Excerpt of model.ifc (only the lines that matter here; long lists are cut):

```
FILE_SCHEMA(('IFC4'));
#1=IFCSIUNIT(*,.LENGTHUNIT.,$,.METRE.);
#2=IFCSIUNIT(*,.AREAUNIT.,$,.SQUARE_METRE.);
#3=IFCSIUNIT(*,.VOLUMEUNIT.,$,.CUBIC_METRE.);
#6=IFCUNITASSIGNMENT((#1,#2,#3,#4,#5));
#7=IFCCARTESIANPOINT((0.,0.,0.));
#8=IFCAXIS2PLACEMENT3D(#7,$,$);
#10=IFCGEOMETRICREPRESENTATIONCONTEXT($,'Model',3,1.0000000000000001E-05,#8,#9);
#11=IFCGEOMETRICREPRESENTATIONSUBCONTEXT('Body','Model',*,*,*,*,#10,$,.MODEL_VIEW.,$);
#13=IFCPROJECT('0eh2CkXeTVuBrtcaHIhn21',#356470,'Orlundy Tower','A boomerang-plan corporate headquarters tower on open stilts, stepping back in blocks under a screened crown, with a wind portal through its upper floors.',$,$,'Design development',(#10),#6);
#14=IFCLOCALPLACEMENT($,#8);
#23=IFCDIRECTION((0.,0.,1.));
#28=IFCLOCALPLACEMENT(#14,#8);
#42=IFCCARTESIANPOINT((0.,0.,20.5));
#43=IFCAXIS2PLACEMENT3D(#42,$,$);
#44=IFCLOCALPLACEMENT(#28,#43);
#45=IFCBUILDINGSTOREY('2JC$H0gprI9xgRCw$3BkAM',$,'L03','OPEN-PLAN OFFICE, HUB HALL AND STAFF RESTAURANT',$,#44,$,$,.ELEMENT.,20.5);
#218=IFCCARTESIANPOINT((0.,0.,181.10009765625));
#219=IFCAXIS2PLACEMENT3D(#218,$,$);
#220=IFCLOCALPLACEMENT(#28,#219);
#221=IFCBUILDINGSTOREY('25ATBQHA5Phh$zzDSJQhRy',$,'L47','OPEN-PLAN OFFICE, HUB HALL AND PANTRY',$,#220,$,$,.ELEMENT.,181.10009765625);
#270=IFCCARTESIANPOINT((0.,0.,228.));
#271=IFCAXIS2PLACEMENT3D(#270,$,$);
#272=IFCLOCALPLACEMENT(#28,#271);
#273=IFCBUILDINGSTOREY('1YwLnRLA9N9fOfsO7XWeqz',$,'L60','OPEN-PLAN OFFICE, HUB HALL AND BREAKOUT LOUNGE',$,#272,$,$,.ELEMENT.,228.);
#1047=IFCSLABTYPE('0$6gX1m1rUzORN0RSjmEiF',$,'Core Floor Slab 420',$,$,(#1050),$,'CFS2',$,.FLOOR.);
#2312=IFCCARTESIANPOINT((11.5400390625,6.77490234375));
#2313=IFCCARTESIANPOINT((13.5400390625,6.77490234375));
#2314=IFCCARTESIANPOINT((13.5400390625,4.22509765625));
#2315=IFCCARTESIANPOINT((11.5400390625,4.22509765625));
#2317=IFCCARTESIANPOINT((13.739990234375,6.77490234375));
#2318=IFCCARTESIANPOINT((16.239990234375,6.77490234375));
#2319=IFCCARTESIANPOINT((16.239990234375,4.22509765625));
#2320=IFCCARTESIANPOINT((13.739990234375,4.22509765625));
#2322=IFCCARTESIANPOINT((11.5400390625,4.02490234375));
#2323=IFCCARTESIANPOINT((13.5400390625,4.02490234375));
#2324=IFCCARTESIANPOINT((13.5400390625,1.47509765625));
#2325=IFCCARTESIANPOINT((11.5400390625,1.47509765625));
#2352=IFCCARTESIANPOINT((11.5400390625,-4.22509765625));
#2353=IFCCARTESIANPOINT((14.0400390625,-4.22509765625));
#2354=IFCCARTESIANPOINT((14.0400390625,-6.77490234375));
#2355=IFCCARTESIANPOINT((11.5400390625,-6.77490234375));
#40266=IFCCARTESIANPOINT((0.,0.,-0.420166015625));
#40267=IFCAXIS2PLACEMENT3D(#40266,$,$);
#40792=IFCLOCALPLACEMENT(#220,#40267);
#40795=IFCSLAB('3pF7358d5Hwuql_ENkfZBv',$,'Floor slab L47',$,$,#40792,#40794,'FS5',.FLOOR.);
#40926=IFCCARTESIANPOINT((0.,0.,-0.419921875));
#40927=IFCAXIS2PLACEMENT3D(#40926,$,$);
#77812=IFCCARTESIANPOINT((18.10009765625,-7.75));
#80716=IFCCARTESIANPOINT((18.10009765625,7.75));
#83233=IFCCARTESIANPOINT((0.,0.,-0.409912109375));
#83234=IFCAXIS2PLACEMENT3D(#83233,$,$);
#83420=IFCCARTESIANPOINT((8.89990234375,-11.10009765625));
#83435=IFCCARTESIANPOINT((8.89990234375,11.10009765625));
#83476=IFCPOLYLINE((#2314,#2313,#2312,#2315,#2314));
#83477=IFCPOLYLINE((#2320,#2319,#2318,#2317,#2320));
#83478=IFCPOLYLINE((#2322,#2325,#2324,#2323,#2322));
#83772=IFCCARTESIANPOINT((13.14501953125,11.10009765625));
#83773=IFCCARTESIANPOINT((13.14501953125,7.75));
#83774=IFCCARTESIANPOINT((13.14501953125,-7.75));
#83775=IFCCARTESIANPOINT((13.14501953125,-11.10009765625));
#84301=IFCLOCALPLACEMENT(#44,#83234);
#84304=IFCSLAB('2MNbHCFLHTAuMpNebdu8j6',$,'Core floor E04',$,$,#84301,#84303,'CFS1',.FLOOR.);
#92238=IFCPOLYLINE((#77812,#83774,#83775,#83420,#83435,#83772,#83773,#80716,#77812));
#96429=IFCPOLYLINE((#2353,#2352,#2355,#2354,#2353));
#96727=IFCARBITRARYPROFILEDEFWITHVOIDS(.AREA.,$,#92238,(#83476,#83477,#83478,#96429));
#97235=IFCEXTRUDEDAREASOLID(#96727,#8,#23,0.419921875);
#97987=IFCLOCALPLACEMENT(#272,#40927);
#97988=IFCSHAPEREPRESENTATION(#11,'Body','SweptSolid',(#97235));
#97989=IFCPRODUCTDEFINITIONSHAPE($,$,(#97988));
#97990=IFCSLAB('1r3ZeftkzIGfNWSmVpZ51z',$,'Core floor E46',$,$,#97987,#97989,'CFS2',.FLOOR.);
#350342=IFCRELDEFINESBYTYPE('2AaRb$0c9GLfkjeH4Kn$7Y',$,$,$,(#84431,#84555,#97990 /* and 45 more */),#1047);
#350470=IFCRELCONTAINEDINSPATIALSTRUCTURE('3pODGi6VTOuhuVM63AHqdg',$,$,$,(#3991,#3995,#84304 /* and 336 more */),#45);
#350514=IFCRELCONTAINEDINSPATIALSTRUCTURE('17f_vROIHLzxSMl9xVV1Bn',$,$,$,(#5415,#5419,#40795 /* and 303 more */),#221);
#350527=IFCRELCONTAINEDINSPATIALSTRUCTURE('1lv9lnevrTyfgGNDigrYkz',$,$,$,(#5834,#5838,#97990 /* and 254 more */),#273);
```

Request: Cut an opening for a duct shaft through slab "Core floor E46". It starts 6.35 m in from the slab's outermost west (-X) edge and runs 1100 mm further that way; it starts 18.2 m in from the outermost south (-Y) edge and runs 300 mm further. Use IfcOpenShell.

```python
import numpy as np
import ifcopenshell
import ifcopenshell.api.feature
import ifcopenshell.api.geometry
import ifcopenshell.api.root
import ifcopenshell.geom
import ifcopenshell.util.placement
import ifcopenshell.util.representation
import ifcopenshell.util.shape
import ifcopenshell.util.unit

model = ifcopenshell.open("model.ifc")
unit_scale = ifcopenshell.util.unit.calculate_unit_scale(model)
settings = ifcopenshell.geom.settings()


def volume(element):
    """Net volume in cubic metres, openings subtracted."""
    shape = ifcopenshell.geom.create_shape(settings, element)
    return ifcopenshell.util.shape.get_volume(shape.geometry)


slab = model.by_guid("1r3ZeftkzIGfNWSmVpZ51z")
before = volume(slab)

# Extent in the slab's own axes, in metres. The edges named are its -X and -Y sides.
slab_shape = ifcopenshell.geom.create_shape(settings, slab)
vertices = ifcopenshell.util.shape.get_vertices(slab_shape.geometry)
x_min, y_min, bottom = vertices.min(axis=0)
top = vertices[:, 2].max()

opening = ifcopenshell.api.root.create_entity(model, ifc_class="IfcOpeningElement", name="Duct shaft opening", predefined_type="OPENING")
context = ifcopenshell.util.representation.get_context(model, "Model", "Body", "MODEL_VIEW")
width, depth = 1.1, 0.3
outline = [(0.0, 0.0), (width, 0.0), (width, depth), (0.0, depth), (0.0, 0.0)]
# Overshoot both faces by 50 mm so the cut is clean.
shape = ifcopenshell.api.geometry.add_slab_representation(
    model, context=context, depth=top - bottom + 0.1, polyline=outline
)
ifcopenshell.api.geometry.assign_representation(model, product=opening, representation=shape)

matrix = ifcopenshell.util.placement.get_local_placement(slab.ObjectPlacement)
matrix[:, 3] = matrix @ np.append(np.array([x_min + 6.35, y_min + 18.2, bottom - 0.05]) / unit_scale, 1.0)
ifcopenshell.api.geometry.edit_object_placement(model, product=opening, matrix=matrix, is_si=False)
ifcopenshell.api.feature.add_feature(model, feature=opening, element=slab)

after = volume(slab)

print(f"slab volume {before:.3f} -> {after:.3f} m3")

model.write("model_rev.ifc")
```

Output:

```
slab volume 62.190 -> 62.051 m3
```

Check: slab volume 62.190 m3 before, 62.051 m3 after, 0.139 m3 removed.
